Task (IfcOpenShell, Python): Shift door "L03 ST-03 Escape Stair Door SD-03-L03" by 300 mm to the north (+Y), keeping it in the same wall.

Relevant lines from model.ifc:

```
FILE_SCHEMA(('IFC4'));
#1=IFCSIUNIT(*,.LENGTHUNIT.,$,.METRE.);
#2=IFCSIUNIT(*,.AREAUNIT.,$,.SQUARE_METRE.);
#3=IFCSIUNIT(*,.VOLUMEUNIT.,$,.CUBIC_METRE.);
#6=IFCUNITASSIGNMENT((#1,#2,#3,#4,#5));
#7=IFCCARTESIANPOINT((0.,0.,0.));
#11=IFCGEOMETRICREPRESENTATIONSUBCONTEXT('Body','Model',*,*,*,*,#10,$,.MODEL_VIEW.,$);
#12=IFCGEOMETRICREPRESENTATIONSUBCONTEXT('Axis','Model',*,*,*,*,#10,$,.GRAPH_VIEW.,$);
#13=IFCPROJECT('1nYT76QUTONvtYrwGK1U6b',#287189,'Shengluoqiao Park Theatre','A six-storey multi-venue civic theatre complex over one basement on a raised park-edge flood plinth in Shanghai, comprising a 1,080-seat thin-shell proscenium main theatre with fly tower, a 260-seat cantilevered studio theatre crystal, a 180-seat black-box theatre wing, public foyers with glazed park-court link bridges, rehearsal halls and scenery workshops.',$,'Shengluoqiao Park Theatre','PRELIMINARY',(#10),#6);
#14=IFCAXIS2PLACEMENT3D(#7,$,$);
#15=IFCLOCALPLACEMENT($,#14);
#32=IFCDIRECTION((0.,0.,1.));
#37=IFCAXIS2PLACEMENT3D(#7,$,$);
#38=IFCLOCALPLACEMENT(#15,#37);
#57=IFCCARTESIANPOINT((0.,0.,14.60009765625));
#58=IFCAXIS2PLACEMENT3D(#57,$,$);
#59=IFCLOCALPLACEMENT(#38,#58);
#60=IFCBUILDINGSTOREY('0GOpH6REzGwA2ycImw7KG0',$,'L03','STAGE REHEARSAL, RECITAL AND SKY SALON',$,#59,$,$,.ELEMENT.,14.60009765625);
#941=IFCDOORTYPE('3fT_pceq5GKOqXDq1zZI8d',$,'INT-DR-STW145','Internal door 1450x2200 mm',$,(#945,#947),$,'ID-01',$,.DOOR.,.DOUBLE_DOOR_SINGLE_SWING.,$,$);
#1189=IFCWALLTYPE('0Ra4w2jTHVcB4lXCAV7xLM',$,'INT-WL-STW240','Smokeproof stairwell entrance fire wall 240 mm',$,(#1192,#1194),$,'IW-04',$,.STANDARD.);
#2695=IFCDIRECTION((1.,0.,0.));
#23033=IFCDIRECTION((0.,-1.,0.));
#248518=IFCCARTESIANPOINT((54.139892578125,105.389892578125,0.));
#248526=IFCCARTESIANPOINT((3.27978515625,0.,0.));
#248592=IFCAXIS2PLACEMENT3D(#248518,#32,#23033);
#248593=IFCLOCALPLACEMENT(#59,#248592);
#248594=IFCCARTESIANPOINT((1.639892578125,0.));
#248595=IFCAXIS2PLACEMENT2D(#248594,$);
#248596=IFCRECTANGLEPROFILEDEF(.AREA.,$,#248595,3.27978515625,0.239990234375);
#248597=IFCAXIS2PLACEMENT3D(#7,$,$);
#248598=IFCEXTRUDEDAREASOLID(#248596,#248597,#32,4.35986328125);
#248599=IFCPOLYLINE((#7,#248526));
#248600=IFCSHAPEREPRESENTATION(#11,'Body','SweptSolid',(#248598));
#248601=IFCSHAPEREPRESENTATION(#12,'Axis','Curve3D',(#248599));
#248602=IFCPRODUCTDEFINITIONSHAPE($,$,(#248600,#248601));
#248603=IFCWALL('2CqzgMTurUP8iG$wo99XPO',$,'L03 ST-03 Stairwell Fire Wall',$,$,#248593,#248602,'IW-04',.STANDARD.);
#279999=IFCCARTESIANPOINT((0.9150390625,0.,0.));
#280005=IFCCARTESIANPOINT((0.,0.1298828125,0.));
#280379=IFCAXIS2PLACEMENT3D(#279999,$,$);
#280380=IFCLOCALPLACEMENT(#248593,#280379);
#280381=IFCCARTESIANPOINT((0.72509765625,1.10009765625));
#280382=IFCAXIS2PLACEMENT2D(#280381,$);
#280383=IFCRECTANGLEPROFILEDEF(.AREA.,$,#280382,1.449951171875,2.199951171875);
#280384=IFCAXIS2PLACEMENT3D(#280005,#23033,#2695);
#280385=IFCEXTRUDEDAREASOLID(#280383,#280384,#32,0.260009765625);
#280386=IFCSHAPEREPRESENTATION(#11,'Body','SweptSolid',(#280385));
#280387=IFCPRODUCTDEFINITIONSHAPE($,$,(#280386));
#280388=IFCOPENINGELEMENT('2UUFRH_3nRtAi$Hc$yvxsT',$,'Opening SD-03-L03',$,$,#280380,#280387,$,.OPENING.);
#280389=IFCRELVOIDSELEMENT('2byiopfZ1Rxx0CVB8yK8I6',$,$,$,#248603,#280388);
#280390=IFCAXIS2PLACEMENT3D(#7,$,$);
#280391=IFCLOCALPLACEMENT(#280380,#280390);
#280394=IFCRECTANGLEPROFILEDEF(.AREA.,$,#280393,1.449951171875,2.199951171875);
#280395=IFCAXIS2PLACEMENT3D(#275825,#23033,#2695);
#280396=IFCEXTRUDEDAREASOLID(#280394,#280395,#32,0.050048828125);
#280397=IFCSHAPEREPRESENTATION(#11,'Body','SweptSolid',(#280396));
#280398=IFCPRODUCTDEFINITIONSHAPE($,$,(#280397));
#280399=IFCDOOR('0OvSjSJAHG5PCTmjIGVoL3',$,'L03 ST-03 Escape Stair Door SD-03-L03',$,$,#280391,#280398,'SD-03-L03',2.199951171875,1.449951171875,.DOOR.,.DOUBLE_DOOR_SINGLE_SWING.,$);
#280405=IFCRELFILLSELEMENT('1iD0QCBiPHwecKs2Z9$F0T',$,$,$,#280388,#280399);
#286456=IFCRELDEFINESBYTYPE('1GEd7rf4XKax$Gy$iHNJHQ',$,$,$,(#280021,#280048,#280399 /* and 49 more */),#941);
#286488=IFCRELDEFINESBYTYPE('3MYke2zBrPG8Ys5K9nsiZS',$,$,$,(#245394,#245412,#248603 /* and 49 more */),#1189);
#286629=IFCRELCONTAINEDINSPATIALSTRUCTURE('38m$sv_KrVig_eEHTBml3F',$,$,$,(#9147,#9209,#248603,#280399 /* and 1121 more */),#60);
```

```python
import ifcopenshell
import ifcopenshell.api.geometry
import ifcopenshell.util.placement

model = ifcopenshell.open("model.ifc")

door = model.by_guid("0OvSjSJAHG5PCTmjIGVoL3")
opening = door.FillsVoids[0].RelatingOpeningElement
wall = opening.VoidsElements[0].RelatingBuildingElement

wall_matrix = ifcopenshell.util.placement.get_local_placement(wall.ObjectPlacement)
shift = wall_matrix[:3, 0] * -0.3
before = ifcopenshell.util.placement.get_local_placement(door.ObjectPlacement)[:3, 3].copy()

# The door is placed relative to its opening, so it follows when the opening moves.
matrix = ifcopenshell.util.placement.get_local_placement(opening.ObjectPlacement)
matrix[:3, 3] += shift
ifcopenshell.api.geometry.edit_object_placement(
    model, product=opening, matrix=matrix, is_si=False, should_transform_children=True
)

after = ifcopenshell.util.placement.get_local_placement(door.ObjectPlacement)[:3, 3]
print("door moved by", (after - before).round(3) + 0.0)

model.write("model_v2.ifc")
```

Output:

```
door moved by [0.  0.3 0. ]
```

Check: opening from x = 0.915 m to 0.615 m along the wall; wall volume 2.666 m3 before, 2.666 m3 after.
